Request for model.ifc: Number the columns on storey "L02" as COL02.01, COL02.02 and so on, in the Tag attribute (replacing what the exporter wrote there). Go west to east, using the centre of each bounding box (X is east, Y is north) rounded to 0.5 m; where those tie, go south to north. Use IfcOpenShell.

First a look at what the model holds.

```python
import ifcopenshell
import ifcopenshell.util.element
import ifcopenshell.util.placement

model = ifcopenshell.open("model.ifc")
print(model.schema)
storey = next(s for s in model.by_type("IfcBuildingStorey") if s.Name == "L02")
columns = [e for e in ifcopenshell.util.element.get_decomposition(storey) if e.is_a("IfcColumn")]
for e in sorted(columns, key=lambda e: e.id()):
    origin = ifcopenshell.util.placement.get_local_placement(e.ObjectPlacement)[:3, 3]
    print(e.id(), e.Tag, e.Name, origin.round(2) + 0.0, sep=" | ")
```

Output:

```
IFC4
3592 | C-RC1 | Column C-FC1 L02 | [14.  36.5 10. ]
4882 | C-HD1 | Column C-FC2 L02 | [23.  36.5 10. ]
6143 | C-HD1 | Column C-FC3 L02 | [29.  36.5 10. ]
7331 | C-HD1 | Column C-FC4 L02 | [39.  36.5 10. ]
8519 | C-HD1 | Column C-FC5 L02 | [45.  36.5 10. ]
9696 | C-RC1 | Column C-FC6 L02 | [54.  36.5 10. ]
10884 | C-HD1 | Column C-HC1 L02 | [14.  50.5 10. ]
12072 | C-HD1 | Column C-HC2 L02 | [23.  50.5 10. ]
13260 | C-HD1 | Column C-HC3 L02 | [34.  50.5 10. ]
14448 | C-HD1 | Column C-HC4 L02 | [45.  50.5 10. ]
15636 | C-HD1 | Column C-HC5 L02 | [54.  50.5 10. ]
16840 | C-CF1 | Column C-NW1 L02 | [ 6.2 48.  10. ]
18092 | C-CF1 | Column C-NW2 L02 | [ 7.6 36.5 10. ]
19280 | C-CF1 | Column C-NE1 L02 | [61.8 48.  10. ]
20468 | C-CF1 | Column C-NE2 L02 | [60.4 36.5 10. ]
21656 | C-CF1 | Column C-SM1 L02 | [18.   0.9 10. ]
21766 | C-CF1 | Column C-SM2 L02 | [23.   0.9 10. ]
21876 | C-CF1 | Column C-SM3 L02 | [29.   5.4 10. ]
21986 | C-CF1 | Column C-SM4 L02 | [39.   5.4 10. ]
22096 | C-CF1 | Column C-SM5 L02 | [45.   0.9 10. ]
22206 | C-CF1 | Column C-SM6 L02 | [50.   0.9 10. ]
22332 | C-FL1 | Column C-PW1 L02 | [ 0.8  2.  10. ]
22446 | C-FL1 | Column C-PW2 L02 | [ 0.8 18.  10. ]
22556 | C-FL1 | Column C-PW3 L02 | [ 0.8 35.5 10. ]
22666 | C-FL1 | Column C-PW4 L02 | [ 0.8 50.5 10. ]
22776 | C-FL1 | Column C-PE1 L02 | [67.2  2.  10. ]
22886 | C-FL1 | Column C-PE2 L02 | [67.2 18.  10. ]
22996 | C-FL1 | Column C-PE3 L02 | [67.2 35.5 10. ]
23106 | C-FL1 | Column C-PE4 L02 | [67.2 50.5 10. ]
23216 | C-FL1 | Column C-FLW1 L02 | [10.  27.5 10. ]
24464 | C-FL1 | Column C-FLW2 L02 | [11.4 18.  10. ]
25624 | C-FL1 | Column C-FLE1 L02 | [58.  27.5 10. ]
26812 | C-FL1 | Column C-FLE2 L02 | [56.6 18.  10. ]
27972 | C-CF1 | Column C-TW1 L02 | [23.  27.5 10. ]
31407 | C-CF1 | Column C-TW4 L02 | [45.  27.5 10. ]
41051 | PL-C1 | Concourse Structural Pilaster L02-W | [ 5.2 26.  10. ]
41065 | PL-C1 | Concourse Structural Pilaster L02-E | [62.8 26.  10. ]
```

```python
import ifcopenshell
import ifcopenshell.geom
import ifcopenshell.util.element
import ifcopenshell.util.shape

model = ifcopenshell.open("model.ifc")
settings = ifcopenshell.geom.settings()
settings.set("use-world-coords", True)


def centre(element):
    shape = ifcopenshell.geom.create_shape(settings, element)
    return ifcopenshell.util.shape.get_bbox_centroid(shape.geometry)


storey = next(s for s in model.by_type("IfcBuildingStorey") if s.Name == "L02")
columns = [e for e in ifcopenshell.util.element.get_decomposition(storey) if e.is_a("IfcColumn")]

# Insertion points can sit at a corner or the storey origin, so sort by the geometry (in metres).
centres = {e: centre(e) for e in columns}
columns.sort(key=lambda e: (round(centres[e][0] / 0.5), centres[e][1]))

for i, e in enumerate(columns, start=1):
    number = f"COL02.{i:02d}"
    e.Tag = number
    print(e.id(), number)

model.write("model_edited.ifc")
```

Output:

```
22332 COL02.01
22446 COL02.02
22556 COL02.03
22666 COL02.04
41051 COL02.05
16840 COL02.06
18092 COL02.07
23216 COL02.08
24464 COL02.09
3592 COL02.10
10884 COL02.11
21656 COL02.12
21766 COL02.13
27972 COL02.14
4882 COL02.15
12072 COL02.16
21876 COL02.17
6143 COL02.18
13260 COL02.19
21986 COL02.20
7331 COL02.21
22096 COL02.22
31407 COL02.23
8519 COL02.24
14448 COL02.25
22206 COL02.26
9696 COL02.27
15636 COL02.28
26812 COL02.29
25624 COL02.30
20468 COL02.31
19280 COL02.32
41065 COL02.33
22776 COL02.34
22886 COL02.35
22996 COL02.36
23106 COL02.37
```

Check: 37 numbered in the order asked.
